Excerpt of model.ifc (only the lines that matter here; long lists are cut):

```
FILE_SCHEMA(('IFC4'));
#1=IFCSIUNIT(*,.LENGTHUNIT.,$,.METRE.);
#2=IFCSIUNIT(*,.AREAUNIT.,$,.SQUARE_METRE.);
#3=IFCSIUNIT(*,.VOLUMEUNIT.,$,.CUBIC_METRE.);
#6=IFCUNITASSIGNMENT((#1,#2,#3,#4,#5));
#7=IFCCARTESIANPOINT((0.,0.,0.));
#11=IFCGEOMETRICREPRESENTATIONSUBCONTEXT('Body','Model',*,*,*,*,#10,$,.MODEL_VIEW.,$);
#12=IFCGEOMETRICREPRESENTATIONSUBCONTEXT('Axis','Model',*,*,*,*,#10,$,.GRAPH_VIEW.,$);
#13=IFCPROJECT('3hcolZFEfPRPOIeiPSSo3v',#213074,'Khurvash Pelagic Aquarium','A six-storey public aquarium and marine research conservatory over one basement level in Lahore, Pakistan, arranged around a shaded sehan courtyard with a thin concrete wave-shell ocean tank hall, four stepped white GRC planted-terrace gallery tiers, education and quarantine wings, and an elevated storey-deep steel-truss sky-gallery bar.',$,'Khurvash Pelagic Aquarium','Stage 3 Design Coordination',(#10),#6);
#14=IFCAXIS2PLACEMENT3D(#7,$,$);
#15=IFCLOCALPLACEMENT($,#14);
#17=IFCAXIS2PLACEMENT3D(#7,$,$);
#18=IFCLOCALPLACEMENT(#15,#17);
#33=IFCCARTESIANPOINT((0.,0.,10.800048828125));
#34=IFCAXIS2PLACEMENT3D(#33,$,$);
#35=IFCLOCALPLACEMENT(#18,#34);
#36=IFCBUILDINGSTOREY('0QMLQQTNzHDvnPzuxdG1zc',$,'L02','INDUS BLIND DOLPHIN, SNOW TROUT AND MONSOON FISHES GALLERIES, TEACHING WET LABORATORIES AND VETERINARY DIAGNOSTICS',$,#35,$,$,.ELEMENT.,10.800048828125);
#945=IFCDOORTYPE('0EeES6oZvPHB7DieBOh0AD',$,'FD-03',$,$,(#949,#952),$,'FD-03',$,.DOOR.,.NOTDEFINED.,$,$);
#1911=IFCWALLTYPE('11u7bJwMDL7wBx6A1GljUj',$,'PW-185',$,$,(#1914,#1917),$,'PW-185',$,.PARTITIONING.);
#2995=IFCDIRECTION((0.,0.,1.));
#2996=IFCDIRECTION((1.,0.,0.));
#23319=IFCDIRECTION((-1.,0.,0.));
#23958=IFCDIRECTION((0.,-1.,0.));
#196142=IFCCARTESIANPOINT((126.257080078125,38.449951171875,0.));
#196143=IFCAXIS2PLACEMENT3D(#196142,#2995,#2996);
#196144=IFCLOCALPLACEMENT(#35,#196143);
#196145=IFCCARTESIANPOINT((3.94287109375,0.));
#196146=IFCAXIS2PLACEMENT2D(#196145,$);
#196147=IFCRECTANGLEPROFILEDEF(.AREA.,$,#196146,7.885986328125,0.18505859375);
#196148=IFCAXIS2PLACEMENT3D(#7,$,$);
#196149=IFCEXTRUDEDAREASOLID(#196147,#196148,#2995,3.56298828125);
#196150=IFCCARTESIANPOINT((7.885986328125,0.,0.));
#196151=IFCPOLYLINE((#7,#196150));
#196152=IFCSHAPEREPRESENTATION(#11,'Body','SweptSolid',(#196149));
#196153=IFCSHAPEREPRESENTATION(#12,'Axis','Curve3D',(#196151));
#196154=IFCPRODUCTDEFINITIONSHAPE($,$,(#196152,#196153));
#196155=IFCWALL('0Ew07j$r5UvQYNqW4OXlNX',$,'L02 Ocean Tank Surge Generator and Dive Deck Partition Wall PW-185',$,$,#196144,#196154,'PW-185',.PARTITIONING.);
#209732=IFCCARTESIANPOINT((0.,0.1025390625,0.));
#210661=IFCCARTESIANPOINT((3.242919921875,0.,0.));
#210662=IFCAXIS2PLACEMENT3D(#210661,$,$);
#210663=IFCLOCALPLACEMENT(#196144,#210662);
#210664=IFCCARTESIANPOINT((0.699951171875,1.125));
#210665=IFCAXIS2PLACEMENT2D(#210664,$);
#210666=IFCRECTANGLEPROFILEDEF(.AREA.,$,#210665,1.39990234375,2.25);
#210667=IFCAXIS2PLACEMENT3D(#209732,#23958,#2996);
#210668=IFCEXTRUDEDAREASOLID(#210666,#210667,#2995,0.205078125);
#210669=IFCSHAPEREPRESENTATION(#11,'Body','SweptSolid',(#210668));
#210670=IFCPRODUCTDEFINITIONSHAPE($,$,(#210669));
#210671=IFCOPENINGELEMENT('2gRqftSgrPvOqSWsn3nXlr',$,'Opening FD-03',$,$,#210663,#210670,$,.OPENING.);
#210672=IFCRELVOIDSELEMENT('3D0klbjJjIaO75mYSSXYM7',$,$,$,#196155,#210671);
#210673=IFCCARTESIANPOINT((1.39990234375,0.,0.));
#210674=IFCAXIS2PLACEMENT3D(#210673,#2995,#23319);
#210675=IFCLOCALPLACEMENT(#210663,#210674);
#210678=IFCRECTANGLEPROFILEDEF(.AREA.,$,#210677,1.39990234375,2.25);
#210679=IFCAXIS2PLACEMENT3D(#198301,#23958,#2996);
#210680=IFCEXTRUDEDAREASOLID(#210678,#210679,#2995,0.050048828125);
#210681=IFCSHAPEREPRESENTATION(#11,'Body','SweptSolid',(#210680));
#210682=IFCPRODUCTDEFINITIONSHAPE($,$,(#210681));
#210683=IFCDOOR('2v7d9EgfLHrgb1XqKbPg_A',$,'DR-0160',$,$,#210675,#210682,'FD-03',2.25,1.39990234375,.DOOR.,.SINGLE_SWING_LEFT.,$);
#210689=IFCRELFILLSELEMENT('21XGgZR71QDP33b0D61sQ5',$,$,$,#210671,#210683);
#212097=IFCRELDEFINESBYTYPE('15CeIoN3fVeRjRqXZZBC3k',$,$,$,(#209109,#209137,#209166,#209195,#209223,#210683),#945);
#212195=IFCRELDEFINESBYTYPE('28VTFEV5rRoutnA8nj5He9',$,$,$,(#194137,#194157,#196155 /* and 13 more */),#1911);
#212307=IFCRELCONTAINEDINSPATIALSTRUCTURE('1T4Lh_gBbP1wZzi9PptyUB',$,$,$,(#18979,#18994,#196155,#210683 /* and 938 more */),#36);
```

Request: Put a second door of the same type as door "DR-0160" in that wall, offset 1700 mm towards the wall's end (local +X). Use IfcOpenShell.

```python
import ifcopenshell
import ifcopenshell.api.feature
import ifcopenshell.api.geometry
import ifcopenshell.api.root
import ifcopenshell.geom
import ifcopenshell.util.element
import ifcopenshell.util.placement
import ifcopenshell.util.shape

model = ifcopenshell.open("model.ifc")
settings = ifcopenshell.geom.settings()


def volume(element):
    """Net volume in cubic metres, openings subtracted."""
    shape = ifcopenshell.geom.create_shape(settings, element)
    return ifcopenshell.util.shape.get_volume(shape.geometry)


door = model.by_guid("2v7d9EgfLHrgb1XqKbPg_A")
opening = door.FillsVoids[0].RelatingOpeningElement
wall = opening.VoidsElements[0].RelatingBuildingElement
before = volume(wall)
shift = ifcopenshell.util.placement.get_local_placement(wall.ObjectPlacement)[:3, 0] * 1.7

# copy_class copies the void relationship, type, container and properties, but no geometry.
new_opening = ifcopenshell.api.root.copy_class(model, product=opening)
new_opening.Representation = ifcopenshell.util.element.copy_deep(
    model, opening.Representation, exclude=["IfcGeometricRepresentationContext", "IfcRepresentationMap"]
)
new_door = ifcopenshell.api.root.copy_class(model, product=door)
new_door.Representation = ifcopenshell.util.element.copy_deep(
    model, door.Representation, exclude=["IfcGeometricRepresentationContext", "IfcRepresentationMap"]
)
new_door.Tag = None
ifcopenshell.api.feature.add_filling(model, opening=new_opening, element=new_door)

for old, new in ((opening, new_opening), (door, new_door)):
    matrix = ifcopenshell.util.placement.get_local_placement(old.ObjectPlacement)
    matrix[:3, 3] += shift
    ifcopenshell.api.geometry.edit_object_placement(model, product=new, matrix=matrix, is_si=False)

after = volume(wall)

print(f"wall volume {before:.3f} -> {after:.3f} m3")

model.write("model_v2.ifc")
```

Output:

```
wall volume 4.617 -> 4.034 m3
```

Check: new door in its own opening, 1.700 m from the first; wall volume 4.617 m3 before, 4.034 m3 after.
